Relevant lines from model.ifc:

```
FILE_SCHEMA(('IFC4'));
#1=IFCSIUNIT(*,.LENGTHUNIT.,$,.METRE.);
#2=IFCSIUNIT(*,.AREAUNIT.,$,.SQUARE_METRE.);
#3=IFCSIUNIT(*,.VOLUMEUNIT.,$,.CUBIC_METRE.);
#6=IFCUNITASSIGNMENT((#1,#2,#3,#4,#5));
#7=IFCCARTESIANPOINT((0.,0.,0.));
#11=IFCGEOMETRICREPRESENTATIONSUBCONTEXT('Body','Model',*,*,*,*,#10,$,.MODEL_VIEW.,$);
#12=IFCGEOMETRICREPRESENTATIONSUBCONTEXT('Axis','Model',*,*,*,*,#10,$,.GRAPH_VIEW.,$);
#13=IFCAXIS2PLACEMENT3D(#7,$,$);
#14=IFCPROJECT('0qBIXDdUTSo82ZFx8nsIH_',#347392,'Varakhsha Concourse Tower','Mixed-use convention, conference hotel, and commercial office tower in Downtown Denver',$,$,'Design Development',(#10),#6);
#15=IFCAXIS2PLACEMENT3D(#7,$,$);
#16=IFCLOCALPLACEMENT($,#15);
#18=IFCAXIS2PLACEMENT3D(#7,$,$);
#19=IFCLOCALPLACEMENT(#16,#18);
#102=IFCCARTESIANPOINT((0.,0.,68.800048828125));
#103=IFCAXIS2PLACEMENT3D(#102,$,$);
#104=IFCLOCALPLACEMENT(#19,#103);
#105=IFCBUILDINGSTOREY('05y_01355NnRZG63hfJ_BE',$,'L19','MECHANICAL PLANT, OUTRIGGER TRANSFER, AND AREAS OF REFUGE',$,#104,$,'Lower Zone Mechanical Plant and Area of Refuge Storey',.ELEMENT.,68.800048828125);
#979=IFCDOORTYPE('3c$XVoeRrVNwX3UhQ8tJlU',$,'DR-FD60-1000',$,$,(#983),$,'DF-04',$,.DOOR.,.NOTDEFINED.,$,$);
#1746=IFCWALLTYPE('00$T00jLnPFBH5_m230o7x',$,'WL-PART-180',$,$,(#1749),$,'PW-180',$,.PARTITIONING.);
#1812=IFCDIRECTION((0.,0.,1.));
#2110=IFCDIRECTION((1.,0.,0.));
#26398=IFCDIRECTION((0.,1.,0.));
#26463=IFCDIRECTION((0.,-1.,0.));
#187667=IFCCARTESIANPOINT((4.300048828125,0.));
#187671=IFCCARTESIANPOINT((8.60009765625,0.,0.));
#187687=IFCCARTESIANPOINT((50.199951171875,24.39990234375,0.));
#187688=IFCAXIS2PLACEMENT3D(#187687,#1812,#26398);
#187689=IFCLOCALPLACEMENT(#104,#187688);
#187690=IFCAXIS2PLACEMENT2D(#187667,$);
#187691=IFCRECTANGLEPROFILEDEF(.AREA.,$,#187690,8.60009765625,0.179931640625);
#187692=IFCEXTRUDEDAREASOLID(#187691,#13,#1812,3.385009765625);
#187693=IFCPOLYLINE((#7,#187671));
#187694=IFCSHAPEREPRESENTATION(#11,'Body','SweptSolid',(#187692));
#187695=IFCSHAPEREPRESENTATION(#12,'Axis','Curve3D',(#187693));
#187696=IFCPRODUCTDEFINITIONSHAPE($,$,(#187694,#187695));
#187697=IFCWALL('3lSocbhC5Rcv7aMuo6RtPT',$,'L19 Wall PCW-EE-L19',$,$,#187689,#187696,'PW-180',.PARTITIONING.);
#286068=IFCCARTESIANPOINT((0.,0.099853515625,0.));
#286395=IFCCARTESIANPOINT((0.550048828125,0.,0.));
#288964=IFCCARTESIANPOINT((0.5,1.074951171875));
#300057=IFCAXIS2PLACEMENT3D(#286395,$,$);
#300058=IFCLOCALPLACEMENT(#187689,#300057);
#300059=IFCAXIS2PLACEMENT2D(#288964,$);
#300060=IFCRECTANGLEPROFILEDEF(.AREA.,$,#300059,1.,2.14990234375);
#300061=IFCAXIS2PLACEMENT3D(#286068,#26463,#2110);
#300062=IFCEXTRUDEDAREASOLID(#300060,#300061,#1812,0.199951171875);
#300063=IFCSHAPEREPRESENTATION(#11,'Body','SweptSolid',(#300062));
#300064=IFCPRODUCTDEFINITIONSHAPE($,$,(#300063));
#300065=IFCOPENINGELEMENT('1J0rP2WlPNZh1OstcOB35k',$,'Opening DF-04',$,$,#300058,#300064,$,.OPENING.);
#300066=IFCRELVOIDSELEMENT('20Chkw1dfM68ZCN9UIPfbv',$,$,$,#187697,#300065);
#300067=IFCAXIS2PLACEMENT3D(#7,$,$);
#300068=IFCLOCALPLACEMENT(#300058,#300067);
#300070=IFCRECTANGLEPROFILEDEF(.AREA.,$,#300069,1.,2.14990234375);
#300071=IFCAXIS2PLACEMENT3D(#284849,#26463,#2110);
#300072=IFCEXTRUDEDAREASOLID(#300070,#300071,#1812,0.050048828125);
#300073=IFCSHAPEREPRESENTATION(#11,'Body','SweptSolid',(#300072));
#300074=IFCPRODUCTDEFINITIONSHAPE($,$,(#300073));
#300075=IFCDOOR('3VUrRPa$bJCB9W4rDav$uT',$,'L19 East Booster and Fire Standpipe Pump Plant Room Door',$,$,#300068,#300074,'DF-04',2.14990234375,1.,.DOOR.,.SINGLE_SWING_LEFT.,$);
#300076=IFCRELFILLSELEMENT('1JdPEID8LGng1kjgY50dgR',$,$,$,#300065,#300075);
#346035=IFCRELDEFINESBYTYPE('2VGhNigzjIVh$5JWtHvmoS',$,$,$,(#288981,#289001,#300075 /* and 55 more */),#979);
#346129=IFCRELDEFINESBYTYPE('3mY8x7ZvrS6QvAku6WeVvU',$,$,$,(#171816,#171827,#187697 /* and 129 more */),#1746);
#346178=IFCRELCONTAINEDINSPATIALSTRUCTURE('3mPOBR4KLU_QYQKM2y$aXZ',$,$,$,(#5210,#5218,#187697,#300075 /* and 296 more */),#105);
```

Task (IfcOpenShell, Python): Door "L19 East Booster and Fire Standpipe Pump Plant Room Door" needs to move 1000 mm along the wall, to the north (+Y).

```python
import ifcopenshell
import ifcopenshell.api.geometry
import ifcopenshell.util.placement
import ifcopenshell.util.unit

model = ifcopenshell.open("model.ifc")
unit_scale = ifcopenshell.util.unit.calculate_unit_scale(model)

door = model.by_id(300075)
opening = door.FillsVoids[0].RelatingOpeningElement
wall = opening.VoidsElements[0].RelatingBuildingElement

wall_matrix = ifcopenshell.util.placement.get_local_placement(wall.ObjectPlacement)
shift = wall_matrix[:3, 0] * 1 / unit_scale
before = ifcopenshell.util.placement.get_local_placement(door.ObjectPlacement)[:3, 3].copy()

# The door is placed relative to its opening, so it follows when the opening moves.
matrix = ifcopenshell.util.placement.get_local_placement(opening.ObjectPlacement)
matrix[:3, 3] += shift
ifcopenshell.api.geometry.edit_object_placement(
    model, product=opening, matrix=matrix, is_si=False, should_transform_children=True
)

after = ifcopenshell.util.placement.get_local_placement(door.ObjectPlacement)[:3, 3]
print("door moved by", (after - before).round(3) + 0.0)

model.write("model_edited.ifc")
```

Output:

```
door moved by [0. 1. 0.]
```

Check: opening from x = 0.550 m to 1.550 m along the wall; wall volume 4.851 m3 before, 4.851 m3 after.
